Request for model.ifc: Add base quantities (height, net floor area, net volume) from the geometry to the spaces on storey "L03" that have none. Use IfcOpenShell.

First a look at what the model holds.

```python
import ifcopenshell
import ifcopenshell.util.element
import ifcopenshell.util.unit

model = ifcopenshell.open("model.ifc")
print(model.schema)
for unit_type in ("LENGTHUNIT", "AREAUNIT", "VOLUMEUNIT"):
    print(unit_type, ifcopenshell.util.unit.calculate_unit_scale(model, unit_type))
storey = next(s for s in model.by_type("IfcBuildingStorey") if s.Name == "L03")
spaces = [e for e in ifcopenshell.util.element.get_decomposition(storey) if e.is_a("IfcSpace")]
for e in sorted(spaces, key=lambda e: e.id()):
    print(e.id(), e.is_a(), e.Name, list(ifcopenshell.util.element.get_psets(e, qtos_only=True)), sep=" | ")
```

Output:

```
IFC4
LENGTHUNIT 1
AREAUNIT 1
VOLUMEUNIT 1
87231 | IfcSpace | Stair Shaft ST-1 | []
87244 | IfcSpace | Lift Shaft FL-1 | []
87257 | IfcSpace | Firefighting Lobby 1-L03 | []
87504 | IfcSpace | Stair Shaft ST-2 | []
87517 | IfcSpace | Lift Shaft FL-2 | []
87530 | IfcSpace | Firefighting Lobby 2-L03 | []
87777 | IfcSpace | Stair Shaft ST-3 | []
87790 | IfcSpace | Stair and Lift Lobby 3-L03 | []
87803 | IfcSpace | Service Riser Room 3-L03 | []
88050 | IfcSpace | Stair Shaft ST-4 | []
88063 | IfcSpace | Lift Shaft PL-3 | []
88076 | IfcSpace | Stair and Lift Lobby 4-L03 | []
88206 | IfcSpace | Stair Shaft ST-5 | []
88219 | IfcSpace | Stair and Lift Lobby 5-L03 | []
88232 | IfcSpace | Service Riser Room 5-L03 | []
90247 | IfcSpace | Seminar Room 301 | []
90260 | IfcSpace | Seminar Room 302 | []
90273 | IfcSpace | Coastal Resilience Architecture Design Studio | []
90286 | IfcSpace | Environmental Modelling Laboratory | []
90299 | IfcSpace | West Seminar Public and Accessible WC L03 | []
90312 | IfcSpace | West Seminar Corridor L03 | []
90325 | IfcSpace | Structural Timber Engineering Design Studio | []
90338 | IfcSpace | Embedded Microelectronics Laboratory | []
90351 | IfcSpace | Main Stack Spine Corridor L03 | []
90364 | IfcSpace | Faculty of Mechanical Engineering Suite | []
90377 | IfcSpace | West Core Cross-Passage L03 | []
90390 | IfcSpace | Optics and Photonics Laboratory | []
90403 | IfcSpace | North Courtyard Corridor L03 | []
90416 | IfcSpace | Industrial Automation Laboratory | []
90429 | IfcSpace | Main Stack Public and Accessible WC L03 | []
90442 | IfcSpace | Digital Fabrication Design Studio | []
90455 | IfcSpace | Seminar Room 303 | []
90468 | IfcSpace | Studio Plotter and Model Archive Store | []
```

```python
import ifcopenshell
import ifcopenshell.api.pset
import ifcopenshell.geom
import ifcopenshell.util.element
import ifcopenshell.util.shape
import ifcopenshell.util.unit

model = ifcopenshell.open("model.ifc")
unit_scale = ifcopenshell.util.unit.calculate_unit_scale(model)
area_scale = ifcopenshell.util.unit.calculate_unit_scale(model, "AREAUNIT")
volume_scale = ifcopenshell.util.unit.calculate_unit_scale(model, "VOLUMEUNIT")
settings = ifcopenshell.geom.settings()

storey = next(s for s in model.by_type("IfcBuildingStorey") if s.Name == "L03")
spaces = [e for e in ifcopenshell.util.element.get_decomposition(storey) if e.is_a("IfcSpace")]

for e in sorted(spaces, key=lambda e: e.id()):
    if ifcopenshell.util.element.get_psets(e, qtos_only=True, should_inherit=False):
        continue
    # Geometry comes back in metres, in the element's own axes.
    shape = ifcopenshell.geom.create_shape(settings, e)
    values = {
        "Height": ifcopenshell.util.shape.get_z(shape.geometry) / unit_scale,
        "NetFloorArea": ifcopenshell.util.shape.get_footprint_area(shape.geometry) / area_scale,
        "NetVolume": ifcopenshell.util.shape.get_volume(shape.geometry) / volume_scale,
    }
    qto = ifcopenshell.api.pset.add_qto(model, product=e, name="Qto_SpaceBaseQuantities")
    ifcopenshell.api.pset.edit_qto(model, qto=qto, properties=values)
    print(e.id(), {k: round(v, 3) for k, v in values.items()})

model.write("model-out.ifc")
```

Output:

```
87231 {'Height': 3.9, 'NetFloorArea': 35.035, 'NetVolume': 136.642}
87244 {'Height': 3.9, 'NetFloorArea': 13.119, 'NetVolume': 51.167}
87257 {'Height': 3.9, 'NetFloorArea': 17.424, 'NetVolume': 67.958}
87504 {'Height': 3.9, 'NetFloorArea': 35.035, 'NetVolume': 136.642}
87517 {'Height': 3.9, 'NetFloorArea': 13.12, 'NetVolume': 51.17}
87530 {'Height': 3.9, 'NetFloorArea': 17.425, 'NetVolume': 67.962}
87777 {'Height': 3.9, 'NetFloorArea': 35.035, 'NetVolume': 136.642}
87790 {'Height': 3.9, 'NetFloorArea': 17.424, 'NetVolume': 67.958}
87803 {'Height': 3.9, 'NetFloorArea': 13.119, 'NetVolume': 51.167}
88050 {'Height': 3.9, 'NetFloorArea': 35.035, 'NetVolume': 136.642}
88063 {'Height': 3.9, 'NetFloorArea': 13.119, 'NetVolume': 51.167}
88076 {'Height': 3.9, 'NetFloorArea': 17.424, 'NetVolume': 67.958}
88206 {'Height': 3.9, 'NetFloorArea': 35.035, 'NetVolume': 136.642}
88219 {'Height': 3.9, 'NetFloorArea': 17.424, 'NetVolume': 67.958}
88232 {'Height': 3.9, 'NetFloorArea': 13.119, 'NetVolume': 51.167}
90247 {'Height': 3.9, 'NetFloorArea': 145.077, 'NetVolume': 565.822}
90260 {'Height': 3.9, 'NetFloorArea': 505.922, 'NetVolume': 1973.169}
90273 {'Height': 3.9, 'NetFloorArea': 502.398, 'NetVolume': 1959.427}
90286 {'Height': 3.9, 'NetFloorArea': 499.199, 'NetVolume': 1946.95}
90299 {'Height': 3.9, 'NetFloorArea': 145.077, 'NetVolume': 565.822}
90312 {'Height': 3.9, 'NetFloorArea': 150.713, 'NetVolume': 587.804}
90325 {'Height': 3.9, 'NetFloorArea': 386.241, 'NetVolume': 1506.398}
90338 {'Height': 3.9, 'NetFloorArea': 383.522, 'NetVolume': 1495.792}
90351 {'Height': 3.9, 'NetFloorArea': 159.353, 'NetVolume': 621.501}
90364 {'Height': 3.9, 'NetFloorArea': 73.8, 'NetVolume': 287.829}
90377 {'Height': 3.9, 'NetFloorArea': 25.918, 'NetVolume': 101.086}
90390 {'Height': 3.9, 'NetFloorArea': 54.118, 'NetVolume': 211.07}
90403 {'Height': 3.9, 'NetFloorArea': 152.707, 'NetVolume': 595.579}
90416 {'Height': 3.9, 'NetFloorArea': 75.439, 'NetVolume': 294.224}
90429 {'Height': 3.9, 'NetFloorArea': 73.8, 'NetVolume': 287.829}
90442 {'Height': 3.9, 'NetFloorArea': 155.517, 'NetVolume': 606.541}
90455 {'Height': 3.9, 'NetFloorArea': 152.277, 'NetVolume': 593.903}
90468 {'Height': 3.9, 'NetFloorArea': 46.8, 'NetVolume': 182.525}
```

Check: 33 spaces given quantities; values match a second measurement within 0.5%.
